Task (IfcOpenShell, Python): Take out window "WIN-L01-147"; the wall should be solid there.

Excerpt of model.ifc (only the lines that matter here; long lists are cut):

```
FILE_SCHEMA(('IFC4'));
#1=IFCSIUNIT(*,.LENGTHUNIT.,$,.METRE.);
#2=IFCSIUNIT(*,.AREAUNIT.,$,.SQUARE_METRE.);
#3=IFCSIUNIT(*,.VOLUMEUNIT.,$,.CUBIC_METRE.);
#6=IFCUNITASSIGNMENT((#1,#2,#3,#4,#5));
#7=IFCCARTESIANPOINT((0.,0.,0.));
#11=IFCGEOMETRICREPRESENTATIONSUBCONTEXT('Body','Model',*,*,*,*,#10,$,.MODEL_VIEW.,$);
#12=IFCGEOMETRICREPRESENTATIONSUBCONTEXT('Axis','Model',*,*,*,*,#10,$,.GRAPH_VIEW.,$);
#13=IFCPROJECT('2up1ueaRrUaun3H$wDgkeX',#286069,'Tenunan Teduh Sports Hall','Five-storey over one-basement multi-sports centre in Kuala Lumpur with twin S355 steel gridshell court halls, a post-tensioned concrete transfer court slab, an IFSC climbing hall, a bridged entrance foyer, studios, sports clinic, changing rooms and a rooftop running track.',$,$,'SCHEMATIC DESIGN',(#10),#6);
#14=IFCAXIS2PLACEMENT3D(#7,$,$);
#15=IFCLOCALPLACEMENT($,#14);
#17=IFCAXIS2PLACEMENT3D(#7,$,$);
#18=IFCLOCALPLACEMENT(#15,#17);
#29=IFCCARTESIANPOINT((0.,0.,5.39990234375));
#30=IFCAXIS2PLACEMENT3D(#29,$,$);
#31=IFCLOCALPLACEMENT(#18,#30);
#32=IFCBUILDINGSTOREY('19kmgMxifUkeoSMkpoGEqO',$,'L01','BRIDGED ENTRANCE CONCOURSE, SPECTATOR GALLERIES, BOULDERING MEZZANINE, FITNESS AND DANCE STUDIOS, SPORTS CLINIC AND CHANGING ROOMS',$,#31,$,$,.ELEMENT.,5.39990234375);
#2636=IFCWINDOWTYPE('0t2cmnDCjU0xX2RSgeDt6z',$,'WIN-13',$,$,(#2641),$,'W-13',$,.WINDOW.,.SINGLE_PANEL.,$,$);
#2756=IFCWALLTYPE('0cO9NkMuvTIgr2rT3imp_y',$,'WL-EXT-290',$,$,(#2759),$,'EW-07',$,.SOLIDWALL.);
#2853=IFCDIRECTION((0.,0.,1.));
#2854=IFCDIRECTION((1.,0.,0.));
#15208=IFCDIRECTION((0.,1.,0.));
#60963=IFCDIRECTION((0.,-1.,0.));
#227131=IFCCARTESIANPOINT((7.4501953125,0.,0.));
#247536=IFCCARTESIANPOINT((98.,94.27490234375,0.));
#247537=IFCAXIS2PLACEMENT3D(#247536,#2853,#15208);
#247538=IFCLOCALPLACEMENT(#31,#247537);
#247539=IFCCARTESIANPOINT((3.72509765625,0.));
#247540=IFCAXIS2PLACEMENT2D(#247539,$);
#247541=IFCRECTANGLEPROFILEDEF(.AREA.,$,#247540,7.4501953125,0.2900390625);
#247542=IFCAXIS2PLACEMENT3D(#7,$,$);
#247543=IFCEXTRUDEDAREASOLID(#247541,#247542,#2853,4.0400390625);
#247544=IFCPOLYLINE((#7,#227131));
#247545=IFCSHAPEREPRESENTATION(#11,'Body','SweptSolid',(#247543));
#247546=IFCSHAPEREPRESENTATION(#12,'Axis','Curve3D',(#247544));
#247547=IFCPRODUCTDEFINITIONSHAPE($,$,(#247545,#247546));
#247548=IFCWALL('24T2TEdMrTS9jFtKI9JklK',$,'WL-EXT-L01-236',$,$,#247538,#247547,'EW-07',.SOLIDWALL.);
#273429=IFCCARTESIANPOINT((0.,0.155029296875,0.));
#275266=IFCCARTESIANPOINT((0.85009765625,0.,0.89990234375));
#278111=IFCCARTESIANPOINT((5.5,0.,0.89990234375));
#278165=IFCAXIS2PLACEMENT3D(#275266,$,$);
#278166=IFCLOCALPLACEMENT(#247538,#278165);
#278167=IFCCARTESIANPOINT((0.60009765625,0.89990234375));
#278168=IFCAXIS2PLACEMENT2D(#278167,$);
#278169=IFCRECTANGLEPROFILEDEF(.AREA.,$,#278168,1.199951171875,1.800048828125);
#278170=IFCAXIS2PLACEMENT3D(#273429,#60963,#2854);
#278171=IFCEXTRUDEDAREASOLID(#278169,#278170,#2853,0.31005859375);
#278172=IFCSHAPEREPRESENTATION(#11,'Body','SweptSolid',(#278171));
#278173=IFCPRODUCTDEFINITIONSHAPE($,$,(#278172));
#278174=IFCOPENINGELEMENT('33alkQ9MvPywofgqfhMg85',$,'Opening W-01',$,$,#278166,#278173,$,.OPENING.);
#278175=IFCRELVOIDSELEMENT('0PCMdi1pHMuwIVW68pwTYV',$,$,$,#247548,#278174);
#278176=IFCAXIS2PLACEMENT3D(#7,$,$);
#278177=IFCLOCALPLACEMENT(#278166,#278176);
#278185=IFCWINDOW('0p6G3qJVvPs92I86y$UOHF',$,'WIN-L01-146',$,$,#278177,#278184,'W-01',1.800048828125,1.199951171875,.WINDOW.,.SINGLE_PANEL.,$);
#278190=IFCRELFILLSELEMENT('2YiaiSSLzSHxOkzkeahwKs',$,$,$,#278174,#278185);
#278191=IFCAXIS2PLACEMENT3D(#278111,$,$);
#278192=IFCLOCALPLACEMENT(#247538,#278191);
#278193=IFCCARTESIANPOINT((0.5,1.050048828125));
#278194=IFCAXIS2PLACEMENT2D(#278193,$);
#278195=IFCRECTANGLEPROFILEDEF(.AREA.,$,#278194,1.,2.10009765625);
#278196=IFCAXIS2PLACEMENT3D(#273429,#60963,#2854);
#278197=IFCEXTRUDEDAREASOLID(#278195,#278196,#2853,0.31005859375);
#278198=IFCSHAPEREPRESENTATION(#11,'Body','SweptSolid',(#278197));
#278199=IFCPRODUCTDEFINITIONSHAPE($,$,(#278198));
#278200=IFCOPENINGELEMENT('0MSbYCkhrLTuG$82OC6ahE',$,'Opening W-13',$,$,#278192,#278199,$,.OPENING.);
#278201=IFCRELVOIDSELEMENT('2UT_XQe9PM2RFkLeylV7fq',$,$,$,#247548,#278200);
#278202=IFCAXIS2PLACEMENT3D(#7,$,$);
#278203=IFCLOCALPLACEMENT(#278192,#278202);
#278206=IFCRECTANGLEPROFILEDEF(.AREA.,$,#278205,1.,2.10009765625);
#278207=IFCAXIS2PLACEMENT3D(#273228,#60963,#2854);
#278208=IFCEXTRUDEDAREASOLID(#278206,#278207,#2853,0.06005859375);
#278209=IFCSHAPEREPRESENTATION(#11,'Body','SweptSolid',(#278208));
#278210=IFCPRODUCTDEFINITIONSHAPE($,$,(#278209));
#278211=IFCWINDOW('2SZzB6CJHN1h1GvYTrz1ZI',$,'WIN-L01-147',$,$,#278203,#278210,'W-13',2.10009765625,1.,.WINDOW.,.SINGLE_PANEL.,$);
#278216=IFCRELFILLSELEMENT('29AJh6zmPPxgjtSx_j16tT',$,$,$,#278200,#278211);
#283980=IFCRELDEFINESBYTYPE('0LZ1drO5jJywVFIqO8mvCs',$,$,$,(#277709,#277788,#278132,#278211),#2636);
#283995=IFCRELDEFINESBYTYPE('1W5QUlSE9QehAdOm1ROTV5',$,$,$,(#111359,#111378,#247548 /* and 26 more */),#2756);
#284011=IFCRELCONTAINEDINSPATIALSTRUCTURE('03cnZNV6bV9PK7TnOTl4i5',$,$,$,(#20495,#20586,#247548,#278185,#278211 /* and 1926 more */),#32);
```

```python
import ifcopenshell
import ifcopenshell.api.feature
import ifcopenshell.api.root
import ifcopenshell.geom
import ifcopenshell.util.shape

model = ifcopenshell.open("model.ifc")
settings = ifcopenshell.geom.settings()


def volume(element):
    """Net volume in cubic metres, openings subtracted."""
    shape = ifcopenshell.geom.create_shape(settings, element)
    return ifcopenshell.util.shape.get_volume(shape.geometry)


window = model.by_guid("2SZzB6CJHN1h1GvYTrz1ZI")
opening = window.FillsVoids[0].RelatingOpeningElement
wall = opening.VoidsElements[0].RelatingBuildingElement
before = volume(wall)

ifcopenshell.api.root.remove_product(model, product=window)
ifcopenshell.api.feature.remove_feature(model, feature=opening)

after = volume(wall)

print(f"wall volume {before:.3f} -> {after:.3f} m3")

model.write("model_rev.ifc")
```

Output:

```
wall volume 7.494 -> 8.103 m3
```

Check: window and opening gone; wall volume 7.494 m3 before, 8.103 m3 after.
